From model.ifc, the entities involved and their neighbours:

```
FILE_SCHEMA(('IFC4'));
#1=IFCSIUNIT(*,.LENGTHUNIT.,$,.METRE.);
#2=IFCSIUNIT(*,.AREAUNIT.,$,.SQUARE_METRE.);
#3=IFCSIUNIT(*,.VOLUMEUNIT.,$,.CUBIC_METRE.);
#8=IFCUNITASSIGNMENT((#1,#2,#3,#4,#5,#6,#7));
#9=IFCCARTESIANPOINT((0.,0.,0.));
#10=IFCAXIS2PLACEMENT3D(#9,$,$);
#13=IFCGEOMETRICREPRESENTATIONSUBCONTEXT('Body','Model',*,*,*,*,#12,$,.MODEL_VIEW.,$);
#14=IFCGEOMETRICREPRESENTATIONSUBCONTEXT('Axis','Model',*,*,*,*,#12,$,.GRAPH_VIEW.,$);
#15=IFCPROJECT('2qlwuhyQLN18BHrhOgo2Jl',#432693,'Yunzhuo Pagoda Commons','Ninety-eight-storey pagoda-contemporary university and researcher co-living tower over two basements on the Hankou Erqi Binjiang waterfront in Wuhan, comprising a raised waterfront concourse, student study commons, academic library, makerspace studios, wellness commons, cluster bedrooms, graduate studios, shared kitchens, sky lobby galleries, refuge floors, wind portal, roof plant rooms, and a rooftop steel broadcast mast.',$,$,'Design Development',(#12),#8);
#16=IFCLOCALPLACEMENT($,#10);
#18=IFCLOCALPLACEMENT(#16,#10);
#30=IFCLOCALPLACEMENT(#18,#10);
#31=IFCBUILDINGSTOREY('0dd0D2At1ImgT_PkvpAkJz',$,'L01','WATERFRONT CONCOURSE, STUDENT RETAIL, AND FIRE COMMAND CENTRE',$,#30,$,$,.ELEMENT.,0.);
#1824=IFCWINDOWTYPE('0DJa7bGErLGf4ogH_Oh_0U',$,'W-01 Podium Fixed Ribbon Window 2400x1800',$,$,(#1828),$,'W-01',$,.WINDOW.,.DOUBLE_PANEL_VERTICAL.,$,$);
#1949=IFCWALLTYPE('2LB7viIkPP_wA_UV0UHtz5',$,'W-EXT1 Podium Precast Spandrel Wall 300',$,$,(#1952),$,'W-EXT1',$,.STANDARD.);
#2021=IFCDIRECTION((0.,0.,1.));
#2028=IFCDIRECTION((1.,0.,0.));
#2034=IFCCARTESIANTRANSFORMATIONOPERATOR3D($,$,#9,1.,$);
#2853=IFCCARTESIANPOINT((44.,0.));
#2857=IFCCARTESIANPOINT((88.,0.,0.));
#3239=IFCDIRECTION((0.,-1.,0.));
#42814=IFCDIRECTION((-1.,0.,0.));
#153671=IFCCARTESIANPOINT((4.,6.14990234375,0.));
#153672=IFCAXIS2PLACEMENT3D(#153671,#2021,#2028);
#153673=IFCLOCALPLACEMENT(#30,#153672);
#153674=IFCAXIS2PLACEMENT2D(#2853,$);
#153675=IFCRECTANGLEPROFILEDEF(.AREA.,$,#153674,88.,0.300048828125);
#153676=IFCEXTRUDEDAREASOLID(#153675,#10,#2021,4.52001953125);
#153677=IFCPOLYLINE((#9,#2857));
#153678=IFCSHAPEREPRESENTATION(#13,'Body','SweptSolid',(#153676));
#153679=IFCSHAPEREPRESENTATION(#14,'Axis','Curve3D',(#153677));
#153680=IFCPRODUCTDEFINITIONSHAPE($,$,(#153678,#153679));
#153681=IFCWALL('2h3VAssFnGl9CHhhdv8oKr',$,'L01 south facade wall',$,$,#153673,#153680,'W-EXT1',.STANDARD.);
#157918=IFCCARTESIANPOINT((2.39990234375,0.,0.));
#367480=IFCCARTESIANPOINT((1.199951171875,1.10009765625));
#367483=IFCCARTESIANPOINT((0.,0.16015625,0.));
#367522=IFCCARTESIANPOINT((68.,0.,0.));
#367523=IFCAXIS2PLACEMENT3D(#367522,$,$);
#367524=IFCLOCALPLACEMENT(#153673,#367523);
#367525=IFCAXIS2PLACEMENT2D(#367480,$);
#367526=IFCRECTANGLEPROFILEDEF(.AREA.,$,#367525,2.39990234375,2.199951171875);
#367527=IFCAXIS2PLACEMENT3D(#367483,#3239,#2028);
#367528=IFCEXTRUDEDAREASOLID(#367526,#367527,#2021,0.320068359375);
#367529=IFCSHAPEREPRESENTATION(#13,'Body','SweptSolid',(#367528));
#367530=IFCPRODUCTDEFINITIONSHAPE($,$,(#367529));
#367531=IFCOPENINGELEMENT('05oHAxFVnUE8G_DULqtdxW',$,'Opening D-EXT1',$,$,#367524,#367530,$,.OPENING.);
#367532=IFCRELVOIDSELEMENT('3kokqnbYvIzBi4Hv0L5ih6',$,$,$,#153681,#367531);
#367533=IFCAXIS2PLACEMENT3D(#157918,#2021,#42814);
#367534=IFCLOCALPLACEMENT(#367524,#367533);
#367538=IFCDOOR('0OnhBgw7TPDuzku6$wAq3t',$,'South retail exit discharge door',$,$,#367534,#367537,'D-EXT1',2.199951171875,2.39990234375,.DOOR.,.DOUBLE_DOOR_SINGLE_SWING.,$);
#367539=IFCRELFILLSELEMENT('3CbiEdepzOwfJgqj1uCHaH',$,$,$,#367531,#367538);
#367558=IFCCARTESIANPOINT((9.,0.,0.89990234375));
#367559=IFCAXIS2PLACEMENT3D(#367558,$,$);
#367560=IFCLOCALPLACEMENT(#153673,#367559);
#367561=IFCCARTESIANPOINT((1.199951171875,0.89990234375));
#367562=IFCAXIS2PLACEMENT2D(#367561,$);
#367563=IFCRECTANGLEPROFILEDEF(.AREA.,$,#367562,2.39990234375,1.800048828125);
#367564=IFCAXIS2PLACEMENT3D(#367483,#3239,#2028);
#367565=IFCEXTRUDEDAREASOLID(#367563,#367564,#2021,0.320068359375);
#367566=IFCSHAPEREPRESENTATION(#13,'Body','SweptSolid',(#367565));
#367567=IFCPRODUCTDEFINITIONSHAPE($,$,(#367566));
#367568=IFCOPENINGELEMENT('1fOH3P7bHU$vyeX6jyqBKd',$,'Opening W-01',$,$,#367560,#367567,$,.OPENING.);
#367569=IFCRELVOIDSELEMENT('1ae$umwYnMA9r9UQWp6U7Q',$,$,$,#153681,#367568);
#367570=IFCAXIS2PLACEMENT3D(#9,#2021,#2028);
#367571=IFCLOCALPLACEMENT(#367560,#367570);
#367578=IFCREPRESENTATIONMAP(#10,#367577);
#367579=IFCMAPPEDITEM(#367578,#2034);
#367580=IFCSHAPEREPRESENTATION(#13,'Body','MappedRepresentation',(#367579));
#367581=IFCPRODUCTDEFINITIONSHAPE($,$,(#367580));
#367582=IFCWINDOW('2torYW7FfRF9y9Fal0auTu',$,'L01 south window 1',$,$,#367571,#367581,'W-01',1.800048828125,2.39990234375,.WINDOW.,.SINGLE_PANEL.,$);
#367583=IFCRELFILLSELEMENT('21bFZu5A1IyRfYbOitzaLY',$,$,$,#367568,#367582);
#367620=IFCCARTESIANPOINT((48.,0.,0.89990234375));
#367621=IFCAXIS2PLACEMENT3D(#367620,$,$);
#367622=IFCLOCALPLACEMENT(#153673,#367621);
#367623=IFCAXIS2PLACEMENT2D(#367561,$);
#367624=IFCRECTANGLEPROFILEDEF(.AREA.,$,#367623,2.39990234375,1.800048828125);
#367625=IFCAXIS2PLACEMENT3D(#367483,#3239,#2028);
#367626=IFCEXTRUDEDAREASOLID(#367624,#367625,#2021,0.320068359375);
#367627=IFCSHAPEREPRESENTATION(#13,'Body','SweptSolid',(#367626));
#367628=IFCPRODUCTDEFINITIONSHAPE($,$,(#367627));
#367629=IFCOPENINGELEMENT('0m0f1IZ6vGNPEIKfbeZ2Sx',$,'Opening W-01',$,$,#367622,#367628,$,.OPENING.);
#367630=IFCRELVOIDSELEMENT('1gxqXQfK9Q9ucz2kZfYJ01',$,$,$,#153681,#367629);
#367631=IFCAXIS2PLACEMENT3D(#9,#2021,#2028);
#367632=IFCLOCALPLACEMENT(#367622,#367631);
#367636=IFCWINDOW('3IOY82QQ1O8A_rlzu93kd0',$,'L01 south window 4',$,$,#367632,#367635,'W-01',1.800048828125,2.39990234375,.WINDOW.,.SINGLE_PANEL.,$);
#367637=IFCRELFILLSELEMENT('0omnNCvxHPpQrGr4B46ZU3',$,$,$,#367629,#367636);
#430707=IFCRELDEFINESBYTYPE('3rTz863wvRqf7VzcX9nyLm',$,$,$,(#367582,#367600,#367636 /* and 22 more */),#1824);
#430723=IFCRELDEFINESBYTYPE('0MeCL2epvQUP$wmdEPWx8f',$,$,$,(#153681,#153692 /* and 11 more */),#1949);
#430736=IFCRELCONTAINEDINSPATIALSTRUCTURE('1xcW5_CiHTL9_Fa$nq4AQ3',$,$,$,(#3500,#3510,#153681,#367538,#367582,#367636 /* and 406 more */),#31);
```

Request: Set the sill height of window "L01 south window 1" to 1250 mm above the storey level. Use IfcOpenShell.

```python
import numpy as np
import ifcopenshell
import ifcopenshell.api.geometry
import ifcopenshell.geom
import ifcopenshell.util.element
import ifcopenshell.util.placement
import ifcopenshell.util.shape
import ifcopenshell.util.unit

model = ifcopenshell.open("model.ifc")
unit_scale = ifcopenshell.util.unit.calculate_unit_scale(model)

window = model.by_id(367582)
opening = window.FillsVoids[0].RelatingOpeningElement
storey = ifcopenshell.util.element.get_container(window, ifc_class="IfcBuildingStorey")
level = ifcopenshell.util.placement.get_local_placement(storey.ObjectPlacement)[2, 3]

# The opening's origin need not be at the sill, so measure its lowest point.
shape = ifcopenshell.geom.create_shape(ifcopenshell.geom.settings(), opening)
bottom = ifcopenshell.util.shape.get_shape_bottom_elevation(shape, shape.geometry) / unit_scale
dz = level + 1.25 / unit_scale - bottom

shift = np.array([0.0, 0.0, dz])
# The window is placed relative to its opening, so it follows when the opening moves.
matrix = ifcopenshell.util.placement.get_local_placement(opening.ObjectPlacement)
matrix[:3, 3] += shift
ifcopenshell.api.geometry.edit_object_placement(
    model, product=opening, matrix=matrix, is_si=False, should_transform_children=True
)

print(f"moved by {dz * unit_scale:+.3f} m")

model.write("model_updated.ifc")
```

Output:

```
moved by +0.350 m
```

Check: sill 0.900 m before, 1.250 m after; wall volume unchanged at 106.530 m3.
